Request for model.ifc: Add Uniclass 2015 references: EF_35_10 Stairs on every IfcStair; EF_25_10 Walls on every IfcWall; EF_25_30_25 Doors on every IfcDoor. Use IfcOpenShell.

First a look at what the model holds.

```python
import ifcopenshell

model = ifcopenshell.open("model.ifc")
print(model.schema)
print("classifications:", [c.Name for c in model.by_type("IfcClassification")])
for ifc_class in ("IfcDoor", "IfcRoof", "IfcStair", "IfcWall", "IfcWindow"):
    print(ifc_class, len(model.by_type(ifc_class)))
```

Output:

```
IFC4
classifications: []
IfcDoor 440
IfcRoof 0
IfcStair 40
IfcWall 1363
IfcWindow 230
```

```python
import ifcopenshell
import ifcopenshell.api.classification

model = ifcopenshell.open("model.ifc")

system = ifcopenshell.api.classification.add_classification(model, classification="Uniclass 2015")

codes = {
    "IfcStair": ("EF_35_10", "Stairs"),
    "IfcWall": ("EF_25_10", "Walls"),
    "IfcDoor": ("EF_25_30_25", "Doors"),
}
for ifc_class, (code, name) in codes.items():
    products = model.by_type(ifc_class)
    ifcopenshell.api.classification.add_reference(
        model, products=products, classification=system, identification=code, name=name
    )
    print(code, len(products))

model.write("model_edited.ifc")
```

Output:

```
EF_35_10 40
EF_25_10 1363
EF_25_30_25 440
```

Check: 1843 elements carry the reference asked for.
